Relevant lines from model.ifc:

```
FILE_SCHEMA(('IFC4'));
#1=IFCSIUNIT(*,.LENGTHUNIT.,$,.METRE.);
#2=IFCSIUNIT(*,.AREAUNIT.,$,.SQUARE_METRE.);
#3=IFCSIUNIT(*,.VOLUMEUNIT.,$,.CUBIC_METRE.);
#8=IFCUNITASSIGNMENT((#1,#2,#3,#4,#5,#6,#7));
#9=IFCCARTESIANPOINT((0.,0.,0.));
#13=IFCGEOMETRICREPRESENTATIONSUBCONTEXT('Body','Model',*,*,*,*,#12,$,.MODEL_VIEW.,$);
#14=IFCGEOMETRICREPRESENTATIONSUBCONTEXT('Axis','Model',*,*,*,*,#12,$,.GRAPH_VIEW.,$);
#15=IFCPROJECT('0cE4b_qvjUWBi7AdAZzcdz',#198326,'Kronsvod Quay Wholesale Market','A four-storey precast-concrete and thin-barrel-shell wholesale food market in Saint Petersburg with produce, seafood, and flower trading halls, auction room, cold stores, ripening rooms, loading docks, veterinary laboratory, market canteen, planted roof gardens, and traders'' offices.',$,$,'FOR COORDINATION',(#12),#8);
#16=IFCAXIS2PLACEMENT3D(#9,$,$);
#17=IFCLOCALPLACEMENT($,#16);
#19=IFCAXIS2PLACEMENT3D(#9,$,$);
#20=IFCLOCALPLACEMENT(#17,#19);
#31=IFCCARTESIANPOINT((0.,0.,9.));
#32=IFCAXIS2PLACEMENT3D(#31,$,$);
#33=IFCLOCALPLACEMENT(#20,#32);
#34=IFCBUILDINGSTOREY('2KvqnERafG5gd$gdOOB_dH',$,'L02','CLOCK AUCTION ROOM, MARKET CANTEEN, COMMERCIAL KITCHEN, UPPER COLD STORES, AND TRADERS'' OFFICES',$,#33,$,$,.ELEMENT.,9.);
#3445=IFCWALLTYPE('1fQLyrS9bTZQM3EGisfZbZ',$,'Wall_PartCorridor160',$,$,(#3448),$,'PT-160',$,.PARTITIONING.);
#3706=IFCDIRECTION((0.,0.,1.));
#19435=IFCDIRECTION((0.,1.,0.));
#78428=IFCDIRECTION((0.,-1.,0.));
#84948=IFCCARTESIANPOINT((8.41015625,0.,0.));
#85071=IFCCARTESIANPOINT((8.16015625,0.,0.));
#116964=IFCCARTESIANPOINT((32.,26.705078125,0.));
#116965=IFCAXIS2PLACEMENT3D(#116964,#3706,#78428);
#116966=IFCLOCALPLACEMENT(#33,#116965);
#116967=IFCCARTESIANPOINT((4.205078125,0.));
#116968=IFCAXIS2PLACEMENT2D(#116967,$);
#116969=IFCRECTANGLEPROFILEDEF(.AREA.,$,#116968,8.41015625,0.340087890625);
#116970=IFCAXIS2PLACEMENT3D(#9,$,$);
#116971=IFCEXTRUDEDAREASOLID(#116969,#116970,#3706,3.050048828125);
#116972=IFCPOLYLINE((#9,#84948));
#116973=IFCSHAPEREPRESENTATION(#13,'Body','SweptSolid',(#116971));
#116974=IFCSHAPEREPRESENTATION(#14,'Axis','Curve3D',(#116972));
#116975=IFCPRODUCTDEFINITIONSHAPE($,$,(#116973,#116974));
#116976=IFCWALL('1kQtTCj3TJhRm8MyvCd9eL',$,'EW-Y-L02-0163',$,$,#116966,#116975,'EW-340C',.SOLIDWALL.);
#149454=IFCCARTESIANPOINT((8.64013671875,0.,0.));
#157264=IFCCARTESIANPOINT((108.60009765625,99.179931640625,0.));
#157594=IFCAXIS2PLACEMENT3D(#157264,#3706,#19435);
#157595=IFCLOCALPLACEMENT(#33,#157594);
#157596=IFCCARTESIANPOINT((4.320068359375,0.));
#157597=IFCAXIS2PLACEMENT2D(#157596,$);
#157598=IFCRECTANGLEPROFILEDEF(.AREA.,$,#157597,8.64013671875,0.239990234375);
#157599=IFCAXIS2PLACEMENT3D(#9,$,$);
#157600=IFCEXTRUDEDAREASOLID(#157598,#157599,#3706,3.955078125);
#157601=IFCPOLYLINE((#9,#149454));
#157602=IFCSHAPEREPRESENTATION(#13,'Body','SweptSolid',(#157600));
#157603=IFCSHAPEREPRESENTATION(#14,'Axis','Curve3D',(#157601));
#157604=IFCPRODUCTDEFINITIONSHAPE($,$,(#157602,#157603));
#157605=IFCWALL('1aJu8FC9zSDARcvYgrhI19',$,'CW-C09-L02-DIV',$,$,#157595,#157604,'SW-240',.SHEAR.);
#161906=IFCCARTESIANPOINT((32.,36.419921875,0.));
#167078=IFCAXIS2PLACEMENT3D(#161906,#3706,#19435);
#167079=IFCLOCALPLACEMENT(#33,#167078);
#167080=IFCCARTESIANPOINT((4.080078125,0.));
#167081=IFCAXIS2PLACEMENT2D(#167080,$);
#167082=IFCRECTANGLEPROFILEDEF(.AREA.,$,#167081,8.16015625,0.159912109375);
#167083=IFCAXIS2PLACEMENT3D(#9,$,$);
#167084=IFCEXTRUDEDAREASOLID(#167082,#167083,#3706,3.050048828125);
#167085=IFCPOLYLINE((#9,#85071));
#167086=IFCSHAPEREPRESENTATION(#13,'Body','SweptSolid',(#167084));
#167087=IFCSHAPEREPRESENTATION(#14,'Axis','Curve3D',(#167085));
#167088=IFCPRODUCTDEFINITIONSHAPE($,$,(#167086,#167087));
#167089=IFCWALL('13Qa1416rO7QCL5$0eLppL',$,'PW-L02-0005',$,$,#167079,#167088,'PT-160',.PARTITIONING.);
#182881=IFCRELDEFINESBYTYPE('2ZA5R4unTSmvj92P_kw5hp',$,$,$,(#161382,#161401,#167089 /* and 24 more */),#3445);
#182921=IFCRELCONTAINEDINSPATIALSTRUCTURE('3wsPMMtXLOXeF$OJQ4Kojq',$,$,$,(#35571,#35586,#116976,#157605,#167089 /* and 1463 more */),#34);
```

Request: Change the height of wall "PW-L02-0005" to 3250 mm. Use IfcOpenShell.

```python
import ifcopenshell
import ifcopenshell.geom
import ifcopenshell.util.representation
import ifcopenshell.util.shape

model = ifcopenshell.open("model.ifc")
settings = ifcopenshell.geom.settings()


def volume(element):
    """Net volume in cubic metres, openings subtracted."""
    shape = ifcopenshell.geom.create_shape(settings, element)
    return ifcopenshell.util.shape.get_volume(shape.geometry)


wall = model.by_guid("13Qa1416rO7QCL5$0eLppL")
before = volume(wall)

body = ifcopenshell.util.representation.get_representation(wall, "Model", "Body")
solid = body.Items[0]
old_height = solid.Depth
solid.Depth = 3.25
after = volume(wall)

print(f"height {old_height:g} -> {solid.Depth:g}, volume {before:.3f} -> {after:.3f} m3")

model.write("model_updated.ifc")
```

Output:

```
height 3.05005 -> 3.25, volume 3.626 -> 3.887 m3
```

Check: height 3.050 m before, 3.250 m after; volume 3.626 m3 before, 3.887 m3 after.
